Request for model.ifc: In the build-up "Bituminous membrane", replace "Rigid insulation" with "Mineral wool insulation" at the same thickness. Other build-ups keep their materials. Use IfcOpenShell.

First a look at what the model holds.

```python
import ifcopenshell
import ifcopenshell.util.element

model = ifcopenshell.open("model.ifc")
print(model.schema)
for layer_set in model.by_type("IfcMaterialLayerSet"):
    if layer_set.LayerSetName == "Bituminous membrane":
        for layer in layer_set.MaterialLayers:
            print(layer.id(), layer.Material and layer.Material.Name, layer.LayerThickness, sep=" | ")
        print(len(ifcopenshell.util.element.get_elements_by_material(model, layer_set)), "elements and types use it")
print(sorted(m.Name for m in model.by_type("IfcMaterial") if m.Name)[:60])
```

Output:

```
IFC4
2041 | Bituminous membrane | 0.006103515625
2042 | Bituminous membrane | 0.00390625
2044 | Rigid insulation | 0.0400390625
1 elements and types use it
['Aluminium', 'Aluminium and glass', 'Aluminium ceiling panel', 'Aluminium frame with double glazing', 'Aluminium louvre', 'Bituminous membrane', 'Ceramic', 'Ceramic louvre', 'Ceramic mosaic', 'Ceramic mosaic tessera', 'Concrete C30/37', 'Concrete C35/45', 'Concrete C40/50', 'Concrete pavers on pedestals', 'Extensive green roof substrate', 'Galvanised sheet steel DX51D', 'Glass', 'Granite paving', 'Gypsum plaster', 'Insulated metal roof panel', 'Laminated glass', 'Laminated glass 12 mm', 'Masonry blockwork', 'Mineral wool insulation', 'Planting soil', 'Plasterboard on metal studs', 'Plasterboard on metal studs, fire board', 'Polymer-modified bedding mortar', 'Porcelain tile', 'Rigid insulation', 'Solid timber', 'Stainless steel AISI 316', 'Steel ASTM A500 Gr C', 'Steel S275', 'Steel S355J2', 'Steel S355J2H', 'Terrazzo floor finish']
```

```python
import ifcopenshell
import ifcopenshell.api.material

model = ifcopenshell.open("model.ifc")

layer_set = next(s for s in model.by_type("IfcMaterialLayerSet") if s.LayerSetName == "Bituminous membrane")
layer = next(l for l in layer_set.MaterialLayers if l.Material and l.Material.Name == "Rigid insulation")
material = next(m for m in model.by_type("IfcMaterial") if m.Name == "Mineral wool insulation")

# Point this one layer at the other material; renaming the old one would change it everywhere.
ifcopenshell.api.material.edit_layer(model, layer=layer, attributes={}, material=material)

print([l.Material.Name if l.Material else None for l in layer_set.MaterialLayers])

model.write("model_v2.ifc")
```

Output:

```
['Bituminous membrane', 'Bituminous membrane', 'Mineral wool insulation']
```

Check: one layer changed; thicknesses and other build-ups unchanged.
